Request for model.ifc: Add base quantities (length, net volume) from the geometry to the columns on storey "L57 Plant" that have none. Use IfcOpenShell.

First a look at what the model holds.

```python
import ifcopenshell
import ifcopenshell.util.element
import ifcopenshell.util.unit

model = ifcopenshell.open("model.ifc")
print(model.schema)
for unit_type in ("LENGTHUNIT", "AREAUNIT", "VOLUMEUNIT"):
    print(unit_type, ifcopenshell.util.unit.calculate_unit_scale(model, unit_type))
storey = next(s for s in model.by_type("IfcBuildingStorey") if s.Name == "L57 Plant")
columns = [e for e in ifcopenshell.util.element.get_decomposition(storey) if e.is_a("IfcColumn")]
for e in sorted(columns, key=lambda e: e.id()):
    print(e.id(), e.is_a(), e.Name, list(ifcopenshell.util.element.get_psets(e, qtos_only=True)), sep=" | ")
```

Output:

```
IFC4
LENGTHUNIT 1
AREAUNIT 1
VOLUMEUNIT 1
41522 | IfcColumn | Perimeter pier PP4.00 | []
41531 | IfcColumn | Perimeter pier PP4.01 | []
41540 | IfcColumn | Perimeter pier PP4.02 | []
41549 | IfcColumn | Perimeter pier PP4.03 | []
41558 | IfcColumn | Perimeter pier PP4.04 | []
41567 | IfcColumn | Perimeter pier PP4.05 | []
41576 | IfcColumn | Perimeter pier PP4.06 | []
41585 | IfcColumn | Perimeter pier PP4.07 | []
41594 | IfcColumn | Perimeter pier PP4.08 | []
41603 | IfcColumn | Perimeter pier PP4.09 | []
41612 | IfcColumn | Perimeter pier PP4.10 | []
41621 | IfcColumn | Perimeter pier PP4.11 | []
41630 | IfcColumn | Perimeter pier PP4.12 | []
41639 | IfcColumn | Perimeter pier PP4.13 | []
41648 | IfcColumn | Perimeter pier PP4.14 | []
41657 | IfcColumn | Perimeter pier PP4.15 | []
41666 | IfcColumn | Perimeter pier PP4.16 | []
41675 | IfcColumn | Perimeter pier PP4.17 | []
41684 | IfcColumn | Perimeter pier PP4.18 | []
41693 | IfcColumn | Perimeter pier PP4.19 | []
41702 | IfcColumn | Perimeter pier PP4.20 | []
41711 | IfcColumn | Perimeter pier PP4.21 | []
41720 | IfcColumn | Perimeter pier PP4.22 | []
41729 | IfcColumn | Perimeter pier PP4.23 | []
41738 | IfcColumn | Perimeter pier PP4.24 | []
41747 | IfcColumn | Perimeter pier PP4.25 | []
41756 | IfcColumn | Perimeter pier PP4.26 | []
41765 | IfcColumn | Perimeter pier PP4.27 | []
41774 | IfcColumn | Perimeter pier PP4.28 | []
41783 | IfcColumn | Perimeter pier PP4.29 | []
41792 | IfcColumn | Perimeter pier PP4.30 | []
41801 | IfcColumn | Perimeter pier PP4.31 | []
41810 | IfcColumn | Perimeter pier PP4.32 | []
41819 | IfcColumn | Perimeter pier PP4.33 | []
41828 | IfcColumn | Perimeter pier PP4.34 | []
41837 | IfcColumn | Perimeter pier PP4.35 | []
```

```python
import ifcopenshell
import ifcopenshell.api.pset
import ifcopenshell.geom
import ifcopenshell.util.element
import ifcopenshell.util.shape
import ifcopenshell.util.unit

model = ifcopenshell.open("model.ifc")
unit_scale = ifcopenshell.util.unit.calculate_unit_scale(model)
volume_scale = ifcopenshell.util.unit.calculate_unit_scale(model, "VOLUMEUNIT")
settings = ifcopenshell.geom.settings()

storey = next(s for s in model.by_type("IfcBuildingStorey") if s.Name == "L57 Plant")
columns = [e for e in ifcopenshell.util.element.get_decomposition(storey) if e.is_a("IfcColumn")]

for e in sorted(columns, key=lambda e: e.id()):
    if ifcopenshell.util.element.get_psets(e, qtos_only=True, should_inherit=False):
        continue
    # Geometry comes back in metres, in the element's own axes.
    shape = ifcopenshell.geom.create_shape(settings, e)
    values = {
        "Length": ifcopenshell.util.shape.get_z(shape.geometry) / unit_scale,
        "NetVolume": ifcopenshell.util.shape.get_volume(shape.geometry) / volume_scale,
    }
    qto = ifcopenshell.api.pset.add_qto(model, product=e, name="Qto_ColumnBaseQuantities")
    ifcopenshell.api.pset.edit_qto(model, qto=qto, properties=values)
    print(e.id(), {k: round(v, 3) for k, v in values.items()})

model.write("model-out.ifc")
```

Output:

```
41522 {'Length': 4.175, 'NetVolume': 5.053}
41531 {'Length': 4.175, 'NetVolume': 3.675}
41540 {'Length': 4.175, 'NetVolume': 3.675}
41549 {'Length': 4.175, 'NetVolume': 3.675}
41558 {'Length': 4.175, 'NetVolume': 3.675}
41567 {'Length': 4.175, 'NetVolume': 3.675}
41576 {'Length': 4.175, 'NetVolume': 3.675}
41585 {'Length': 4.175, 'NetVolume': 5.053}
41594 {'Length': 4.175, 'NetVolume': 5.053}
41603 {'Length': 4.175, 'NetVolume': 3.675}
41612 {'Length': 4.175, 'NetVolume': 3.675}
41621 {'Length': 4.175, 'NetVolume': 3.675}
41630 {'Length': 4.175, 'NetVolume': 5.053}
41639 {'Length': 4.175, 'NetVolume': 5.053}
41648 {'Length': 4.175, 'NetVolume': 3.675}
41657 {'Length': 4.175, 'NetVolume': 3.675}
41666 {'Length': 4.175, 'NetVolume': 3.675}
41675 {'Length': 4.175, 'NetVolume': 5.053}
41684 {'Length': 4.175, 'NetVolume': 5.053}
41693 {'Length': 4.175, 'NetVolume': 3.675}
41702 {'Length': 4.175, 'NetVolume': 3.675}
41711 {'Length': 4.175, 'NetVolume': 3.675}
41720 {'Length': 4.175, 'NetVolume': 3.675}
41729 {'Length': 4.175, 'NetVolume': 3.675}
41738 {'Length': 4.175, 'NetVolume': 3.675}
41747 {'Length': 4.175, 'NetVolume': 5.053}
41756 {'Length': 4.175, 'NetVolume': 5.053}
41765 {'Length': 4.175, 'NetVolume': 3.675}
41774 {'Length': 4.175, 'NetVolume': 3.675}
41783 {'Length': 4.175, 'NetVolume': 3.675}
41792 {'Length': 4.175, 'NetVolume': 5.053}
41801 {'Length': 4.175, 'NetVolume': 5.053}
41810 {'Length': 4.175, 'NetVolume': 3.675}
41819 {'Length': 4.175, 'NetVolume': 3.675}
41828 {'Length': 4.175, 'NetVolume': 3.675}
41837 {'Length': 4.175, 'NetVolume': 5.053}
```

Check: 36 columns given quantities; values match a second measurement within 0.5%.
